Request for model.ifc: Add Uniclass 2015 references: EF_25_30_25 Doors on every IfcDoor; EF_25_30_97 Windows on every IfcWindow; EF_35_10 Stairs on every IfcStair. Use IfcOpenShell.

First a look at what the model holds.

```python
import ifcopenshell

model = ifcopenshell.open("model.ifc")
print(model.schema)
print("classifications:", [c.Name for c in model.by_type("IfcClassification")])
for ifc_class in ("IfcDoor", "IfcRoof", "IfcStair", "IfcWall", "IfcWindow"):
    print(ifc_class, len(model.by_type(ifc_class)))
```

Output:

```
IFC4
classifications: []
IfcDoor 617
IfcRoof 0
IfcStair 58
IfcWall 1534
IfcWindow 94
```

```python
import ifcopenshell
import ifcopenshell.api.classification

model = ifcopenshell.open("model.ifc")

system = ifcopenshell.api.classification.add_classification(model, classification="Uniclass 2015")

codes = {
    "IfcDoor": ("EF_25_30_25", "Doors"),
    "IfcWindow": ("EF_25_30_97", "Windows"),
    "IfcStair": ("EF_35_10", "Stairs"),
}
for ifc_class, (code, name) in codes.items():
    products = model.by_type(ifc_class)
    ifcopenshell.api.classification.add_reference(
        model, products=products, classification=system, identification=code, name=name
    )
    print(code, len(products))

model.write("model_updated.ifc")
```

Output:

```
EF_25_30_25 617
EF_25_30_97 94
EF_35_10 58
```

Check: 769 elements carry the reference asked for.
